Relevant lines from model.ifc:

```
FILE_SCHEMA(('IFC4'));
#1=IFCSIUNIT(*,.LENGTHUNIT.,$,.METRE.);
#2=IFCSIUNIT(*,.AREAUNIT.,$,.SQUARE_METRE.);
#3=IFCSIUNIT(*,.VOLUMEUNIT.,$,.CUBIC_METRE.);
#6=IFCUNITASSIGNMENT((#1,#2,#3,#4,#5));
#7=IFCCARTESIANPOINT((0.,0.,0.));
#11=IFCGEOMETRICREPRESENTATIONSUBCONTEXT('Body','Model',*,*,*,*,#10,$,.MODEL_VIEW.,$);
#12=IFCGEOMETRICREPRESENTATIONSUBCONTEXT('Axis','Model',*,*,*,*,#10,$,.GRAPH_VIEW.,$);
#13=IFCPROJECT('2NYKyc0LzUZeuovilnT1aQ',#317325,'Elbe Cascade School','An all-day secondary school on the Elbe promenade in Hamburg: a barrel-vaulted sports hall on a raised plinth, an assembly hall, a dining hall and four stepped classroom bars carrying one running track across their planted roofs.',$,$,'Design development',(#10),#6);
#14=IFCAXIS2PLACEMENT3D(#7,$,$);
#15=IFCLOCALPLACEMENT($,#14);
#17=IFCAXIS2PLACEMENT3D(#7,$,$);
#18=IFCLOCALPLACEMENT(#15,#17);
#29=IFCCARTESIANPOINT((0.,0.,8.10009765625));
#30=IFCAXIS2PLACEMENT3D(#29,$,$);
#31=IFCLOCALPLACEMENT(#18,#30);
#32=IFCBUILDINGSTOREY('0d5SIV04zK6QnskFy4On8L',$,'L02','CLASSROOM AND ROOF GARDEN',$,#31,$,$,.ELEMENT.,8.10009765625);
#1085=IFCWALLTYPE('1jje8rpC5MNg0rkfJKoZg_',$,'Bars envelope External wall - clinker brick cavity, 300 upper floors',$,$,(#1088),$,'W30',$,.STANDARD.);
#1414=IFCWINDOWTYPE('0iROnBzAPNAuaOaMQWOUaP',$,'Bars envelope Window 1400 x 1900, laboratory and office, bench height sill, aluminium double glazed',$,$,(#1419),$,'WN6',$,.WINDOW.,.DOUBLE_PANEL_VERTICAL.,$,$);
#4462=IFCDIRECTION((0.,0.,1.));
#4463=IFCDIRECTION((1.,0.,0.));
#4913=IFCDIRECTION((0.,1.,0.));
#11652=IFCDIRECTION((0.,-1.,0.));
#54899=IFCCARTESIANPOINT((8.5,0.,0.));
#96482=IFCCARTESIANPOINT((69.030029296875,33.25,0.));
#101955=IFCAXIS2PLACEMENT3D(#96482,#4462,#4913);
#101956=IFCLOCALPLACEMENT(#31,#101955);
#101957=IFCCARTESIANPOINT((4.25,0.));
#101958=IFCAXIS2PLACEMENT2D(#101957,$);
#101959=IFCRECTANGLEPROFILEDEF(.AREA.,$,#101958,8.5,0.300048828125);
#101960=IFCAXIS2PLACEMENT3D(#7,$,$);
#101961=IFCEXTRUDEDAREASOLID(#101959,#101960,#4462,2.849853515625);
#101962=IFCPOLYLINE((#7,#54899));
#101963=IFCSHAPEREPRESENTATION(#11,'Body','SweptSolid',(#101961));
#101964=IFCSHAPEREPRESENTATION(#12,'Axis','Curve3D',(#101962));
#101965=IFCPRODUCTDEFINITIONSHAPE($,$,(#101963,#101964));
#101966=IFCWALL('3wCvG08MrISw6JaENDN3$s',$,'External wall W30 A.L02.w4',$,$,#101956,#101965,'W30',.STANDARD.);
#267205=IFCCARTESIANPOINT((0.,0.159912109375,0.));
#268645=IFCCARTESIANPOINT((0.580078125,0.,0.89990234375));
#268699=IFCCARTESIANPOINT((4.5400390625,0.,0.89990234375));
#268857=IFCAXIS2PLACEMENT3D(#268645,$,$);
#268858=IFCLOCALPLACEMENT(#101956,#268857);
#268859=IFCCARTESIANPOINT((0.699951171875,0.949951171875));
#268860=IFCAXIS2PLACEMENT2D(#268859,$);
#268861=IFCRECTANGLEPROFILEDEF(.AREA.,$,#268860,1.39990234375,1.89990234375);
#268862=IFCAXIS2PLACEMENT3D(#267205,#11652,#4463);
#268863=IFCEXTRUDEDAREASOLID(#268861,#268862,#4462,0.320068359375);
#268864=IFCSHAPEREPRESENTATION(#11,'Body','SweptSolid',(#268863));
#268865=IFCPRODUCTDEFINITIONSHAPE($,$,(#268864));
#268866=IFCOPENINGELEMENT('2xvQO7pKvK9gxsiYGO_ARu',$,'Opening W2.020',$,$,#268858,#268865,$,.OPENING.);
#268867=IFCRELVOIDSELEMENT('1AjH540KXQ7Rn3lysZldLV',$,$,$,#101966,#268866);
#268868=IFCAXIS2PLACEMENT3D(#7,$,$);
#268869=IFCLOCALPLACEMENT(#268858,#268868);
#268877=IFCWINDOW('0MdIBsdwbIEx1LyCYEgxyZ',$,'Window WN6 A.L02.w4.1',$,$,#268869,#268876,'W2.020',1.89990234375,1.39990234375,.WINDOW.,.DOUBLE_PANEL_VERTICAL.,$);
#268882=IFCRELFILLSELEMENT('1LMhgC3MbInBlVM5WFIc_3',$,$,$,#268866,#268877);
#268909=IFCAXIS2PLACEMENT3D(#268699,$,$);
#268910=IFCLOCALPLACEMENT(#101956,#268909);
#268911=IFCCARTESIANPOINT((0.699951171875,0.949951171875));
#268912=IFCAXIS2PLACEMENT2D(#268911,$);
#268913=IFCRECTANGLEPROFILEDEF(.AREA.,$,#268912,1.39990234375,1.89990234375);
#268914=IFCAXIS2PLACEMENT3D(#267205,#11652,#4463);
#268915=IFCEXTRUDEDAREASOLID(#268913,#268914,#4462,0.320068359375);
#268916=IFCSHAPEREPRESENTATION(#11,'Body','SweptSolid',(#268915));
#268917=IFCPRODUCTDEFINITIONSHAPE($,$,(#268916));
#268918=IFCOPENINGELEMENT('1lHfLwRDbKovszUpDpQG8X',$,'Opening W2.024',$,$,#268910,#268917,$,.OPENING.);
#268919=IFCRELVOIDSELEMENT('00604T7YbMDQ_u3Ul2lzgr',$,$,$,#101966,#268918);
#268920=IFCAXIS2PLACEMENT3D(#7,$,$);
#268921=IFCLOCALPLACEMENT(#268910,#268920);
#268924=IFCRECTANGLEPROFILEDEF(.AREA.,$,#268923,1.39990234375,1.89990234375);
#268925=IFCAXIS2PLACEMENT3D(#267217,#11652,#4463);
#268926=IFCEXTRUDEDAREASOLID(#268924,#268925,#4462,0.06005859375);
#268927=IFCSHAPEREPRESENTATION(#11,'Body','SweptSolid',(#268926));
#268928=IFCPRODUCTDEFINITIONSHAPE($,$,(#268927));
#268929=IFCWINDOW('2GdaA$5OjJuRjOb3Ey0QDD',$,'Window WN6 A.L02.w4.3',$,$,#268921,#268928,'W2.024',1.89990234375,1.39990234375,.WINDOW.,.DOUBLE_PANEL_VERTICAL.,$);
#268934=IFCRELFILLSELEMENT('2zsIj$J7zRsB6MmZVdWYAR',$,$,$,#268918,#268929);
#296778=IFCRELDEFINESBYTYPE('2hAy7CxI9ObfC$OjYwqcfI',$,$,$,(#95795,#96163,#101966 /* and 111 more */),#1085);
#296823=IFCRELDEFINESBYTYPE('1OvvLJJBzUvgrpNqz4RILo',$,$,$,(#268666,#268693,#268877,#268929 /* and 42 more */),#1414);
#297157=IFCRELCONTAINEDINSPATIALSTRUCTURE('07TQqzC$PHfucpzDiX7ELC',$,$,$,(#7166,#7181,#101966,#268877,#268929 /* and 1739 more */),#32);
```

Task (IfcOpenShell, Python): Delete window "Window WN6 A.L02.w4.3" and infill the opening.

```python
import ifcopenshell
import ifcopenshell.api.feature
import ifcopenshell.api.root
import ifcopenshell.geom
import ifcopenshell.util.shape

model = ifcopenshell.open("model.ifc")
settings = ifcopenshell.geom.settings()


def volume(element):
    """Net volume in cubic metres, openings subtracted."""
    shape = ifcopenshell.geom.create_shape(settings, element)
    return ifcopenshell.util.shape.get_volume(shape.geometry)


window = model.by_guid("2GdaA$5OjJuRjOb3Ey0QDD")
opening = window.FillsVoids[0].RelatingOpeningElement
wall = opening.VoidsElements[0].RelatingBuildingElement
before = volume(wall)

ifcopenshell.api.root.remove_product(model, product=window)
ifcopenshell.api.feature.remove_feature(model, feature=opening)

after = volume(wall)

print(f"wall volume {before:.3f} -> {after:.3f} m3")

model.write("model_updated.ifc")
```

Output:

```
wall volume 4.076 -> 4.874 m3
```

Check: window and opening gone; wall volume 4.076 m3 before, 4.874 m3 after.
